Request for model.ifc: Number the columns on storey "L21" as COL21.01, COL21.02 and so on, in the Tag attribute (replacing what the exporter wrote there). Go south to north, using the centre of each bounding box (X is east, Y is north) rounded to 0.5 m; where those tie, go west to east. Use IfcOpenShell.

First a look at what the model holds.

```python
import ifcopenshell
import ifcopenshell.util.element
import ifcopenshell.util.placement

model = ifcopenshell.open("model.ifc")
print(model.schema)
storey = next(s for s in model.by_type("IfcBuildingStorey") if s.Name == "L21")
columns = [e for e in ifcopenshell.util.element.get_decomposition(storey) if e.is_a("IfcColumn")]
for e in sorted(columns, key=lambda e: e.id()):
    origin = ifcopenshell.util.placement.get_local_placement(e.ObjectPlacement)[:3, 3]
    print(e.id(), e.Tag, e.Name, origin.round(2) + 0.0, sep=" | ")
```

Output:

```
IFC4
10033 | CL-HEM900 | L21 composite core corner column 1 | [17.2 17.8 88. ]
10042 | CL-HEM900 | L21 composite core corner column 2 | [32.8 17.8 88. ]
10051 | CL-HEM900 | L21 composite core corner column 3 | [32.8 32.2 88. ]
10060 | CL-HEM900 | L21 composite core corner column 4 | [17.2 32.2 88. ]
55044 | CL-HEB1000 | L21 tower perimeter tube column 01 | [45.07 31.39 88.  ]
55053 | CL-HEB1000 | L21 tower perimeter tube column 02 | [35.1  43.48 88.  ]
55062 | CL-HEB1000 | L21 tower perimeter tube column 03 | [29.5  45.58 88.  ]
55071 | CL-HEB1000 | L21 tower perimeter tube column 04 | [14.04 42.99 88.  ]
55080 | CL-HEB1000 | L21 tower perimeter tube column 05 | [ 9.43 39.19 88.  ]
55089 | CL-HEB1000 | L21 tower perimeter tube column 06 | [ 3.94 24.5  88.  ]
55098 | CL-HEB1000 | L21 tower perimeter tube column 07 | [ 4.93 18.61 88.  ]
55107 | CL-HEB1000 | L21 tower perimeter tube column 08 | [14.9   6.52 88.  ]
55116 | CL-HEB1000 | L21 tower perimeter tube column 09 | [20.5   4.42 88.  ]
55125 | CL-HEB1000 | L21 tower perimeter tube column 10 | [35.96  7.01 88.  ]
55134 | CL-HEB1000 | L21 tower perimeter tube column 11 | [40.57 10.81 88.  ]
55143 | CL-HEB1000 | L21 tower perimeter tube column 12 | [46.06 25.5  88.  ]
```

```python
import ifcopenshell
import ifcopenshell.geom
import ifcopenshell.util.element
import ifcopenshell.util.shape

model = ifcopenshell.open("model.ifc")
settings = ifcopenshell.geom.settings()
settings.set("use-world-coords", True)


def centre(element):
    shape = ifcopenshell.geom.create_shape(settings, element)
    return ifcopenshell.util.shape.get_bbox_centroid(shape.geometry)


storey = next(s for s in model.by_type("IfcBuildingStorey") if s.Name == "L21")
columns = [e for e in ifcopenshell.util.element.get_decomposition(storey) if e.is_a("IfcColumn")]

# Insertion points can sit at a corner or the storey origin, so sort by the geometry (in metres).
centres = {e: centre(e) for e in columns}
columns.sort(key=lambda e: (round(centres[e][1] / 0.5), centres[e][0]))

for i, e in enumerate(columns, start=1):
    number = f"COL21.{i:02d}"
    e.Tag = number
    print(e.id(), number)

model.write("model_edited.ifc")
```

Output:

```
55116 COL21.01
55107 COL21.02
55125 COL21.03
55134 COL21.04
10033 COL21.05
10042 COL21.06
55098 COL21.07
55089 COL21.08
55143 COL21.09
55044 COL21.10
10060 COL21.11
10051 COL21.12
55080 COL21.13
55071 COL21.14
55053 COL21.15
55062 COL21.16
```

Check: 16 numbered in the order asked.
